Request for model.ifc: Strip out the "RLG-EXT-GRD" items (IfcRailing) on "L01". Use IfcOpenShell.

First a look at what the model holds.

```python
import ifcopenshell
import ifcopenshell.util.element

model = ifcopenshell.open("model.ifc")
print(model.schema)
storey = next(s for s in model.by_type("IfcBuildingStorey") if s.Name == "L01")
railings = [e for e in ifcopenshell.util.element.get_decomposition(storey) if e.is_a("IfcRailing")]
seen = {}
for e in railings:
    element_type = ifcopenshell.util.element.get_type(e)
    name = element_type.Name if element_type not in (None, e) else None
    seen[name] = seen.get(name, 0) + 1
for name, count in sorted(seen.items(), key=str):
    print(count, "x", name)
```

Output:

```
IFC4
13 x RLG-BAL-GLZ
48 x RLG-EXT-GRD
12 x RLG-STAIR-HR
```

```python
import ifcopenshell
import ifcopenshell.api.root
import ifcopenshell.util.element

model = ifcopenshell.open("model.ifc")

storey = next(s for s in model.by_type("IfcBuildingStorey") if s.Name == "L01")
railings = [e for e in ifcopenshell.util.element.get_decomposition(storey) if e.is_a("IfcRailing")]
targets = [e for e in railings if (t := ifcopenshell.util.element.get_type(e)) not in (None, e) and t.Name == "RLG-EXT-GRD"]

for e in targets:
    ifcopenshell.api.root.remove_product(model, product=e)
print(len(targets), "removed")

model.write("model_updated.ifc")
```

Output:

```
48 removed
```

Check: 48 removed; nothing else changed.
